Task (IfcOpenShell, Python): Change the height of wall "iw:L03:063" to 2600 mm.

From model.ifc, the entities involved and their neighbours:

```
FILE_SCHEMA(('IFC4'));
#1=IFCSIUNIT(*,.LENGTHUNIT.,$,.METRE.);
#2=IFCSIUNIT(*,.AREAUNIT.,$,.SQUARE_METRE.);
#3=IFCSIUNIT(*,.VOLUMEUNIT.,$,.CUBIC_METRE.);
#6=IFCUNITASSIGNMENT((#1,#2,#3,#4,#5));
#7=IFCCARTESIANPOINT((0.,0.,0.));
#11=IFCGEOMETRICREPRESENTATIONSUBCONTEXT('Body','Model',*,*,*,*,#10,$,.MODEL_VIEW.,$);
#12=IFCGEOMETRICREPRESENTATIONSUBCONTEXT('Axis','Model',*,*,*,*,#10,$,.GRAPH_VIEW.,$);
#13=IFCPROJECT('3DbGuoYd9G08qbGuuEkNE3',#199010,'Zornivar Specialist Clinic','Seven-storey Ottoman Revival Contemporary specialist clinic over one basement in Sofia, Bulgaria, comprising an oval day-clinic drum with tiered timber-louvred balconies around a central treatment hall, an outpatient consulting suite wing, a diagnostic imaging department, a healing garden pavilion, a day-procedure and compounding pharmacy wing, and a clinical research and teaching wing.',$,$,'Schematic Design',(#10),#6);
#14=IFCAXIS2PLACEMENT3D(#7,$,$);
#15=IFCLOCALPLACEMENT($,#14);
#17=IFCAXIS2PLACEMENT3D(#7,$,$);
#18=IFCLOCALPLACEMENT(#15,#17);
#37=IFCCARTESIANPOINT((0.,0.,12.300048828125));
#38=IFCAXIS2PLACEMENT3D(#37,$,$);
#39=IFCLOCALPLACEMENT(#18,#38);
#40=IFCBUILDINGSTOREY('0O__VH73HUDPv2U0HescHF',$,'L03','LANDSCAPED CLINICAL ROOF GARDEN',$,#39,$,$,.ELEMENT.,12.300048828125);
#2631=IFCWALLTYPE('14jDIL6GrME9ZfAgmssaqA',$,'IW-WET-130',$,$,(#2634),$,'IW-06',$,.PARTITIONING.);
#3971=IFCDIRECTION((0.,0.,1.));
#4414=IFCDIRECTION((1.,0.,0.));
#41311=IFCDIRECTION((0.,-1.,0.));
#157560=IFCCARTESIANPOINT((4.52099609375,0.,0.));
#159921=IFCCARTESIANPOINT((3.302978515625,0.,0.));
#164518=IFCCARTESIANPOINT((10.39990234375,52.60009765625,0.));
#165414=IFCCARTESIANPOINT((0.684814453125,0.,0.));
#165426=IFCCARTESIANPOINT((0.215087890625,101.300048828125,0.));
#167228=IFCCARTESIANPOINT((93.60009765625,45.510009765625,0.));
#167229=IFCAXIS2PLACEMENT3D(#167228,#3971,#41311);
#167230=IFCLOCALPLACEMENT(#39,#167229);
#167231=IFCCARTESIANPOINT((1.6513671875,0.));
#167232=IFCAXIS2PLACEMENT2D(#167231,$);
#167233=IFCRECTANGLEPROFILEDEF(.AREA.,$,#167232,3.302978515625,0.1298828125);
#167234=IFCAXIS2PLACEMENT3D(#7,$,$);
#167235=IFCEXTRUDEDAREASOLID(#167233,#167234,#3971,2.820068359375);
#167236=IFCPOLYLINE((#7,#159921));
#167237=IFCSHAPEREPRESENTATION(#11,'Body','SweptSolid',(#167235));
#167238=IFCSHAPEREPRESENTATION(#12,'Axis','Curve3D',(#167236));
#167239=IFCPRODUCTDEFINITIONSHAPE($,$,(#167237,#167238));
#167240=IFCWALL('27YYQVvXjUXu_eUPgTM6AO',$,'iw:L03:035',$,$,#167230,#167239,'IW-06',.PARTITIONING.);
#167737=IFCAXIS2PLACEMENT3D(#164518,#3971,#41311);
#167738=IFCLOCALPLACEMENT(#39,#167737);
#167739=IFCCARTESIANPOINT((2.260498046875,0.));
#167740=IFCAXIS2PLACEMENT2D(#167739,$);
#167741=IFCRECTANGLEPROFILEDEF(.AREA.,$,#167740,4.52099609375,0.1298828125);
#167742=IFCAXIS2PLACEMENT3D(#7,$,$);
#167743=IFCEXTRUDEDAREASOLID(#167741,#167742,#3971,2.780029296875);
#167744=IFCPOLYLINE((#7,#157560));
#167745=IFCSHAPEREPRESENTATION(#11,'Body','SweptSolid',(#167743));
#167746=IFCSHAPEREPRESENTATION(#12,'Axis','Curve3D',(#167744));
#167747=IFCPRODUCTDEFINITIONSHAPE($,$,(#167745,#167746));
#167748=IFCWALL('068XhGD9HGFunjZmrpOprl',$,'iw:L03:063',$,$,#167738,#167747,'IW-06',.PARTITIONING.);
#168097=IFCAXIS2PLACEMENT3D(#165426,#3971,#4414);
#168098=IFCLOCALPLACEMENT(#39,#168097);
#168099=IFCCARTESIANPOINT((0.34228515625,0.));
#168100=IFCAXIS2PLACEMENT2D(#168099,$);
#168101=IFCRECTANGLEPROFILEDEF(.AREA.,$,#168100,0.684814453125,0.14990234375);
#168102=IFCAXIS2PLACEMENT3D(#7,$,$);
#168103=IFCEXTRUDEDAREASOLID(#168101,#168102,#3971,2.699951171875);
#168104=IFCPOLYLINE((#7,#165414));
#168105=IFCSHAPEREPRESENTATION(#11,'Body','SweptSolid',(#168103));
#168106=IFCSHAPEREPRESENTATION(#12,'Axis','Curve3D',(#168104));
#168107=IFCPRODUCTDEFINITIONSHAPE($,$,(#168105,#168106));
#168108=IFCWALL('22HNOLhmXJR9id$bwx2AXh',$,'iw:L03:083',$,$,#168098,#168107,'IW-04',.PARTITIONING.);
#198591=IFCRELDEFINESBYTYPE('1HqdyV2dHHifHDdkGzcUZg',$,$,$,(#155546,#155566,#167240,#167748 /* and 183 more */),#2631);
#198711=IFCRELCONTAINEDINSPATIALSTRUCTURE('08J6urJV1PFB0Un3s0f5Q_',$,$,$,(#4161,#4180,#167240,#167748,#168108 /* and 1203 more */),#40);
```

```python
import ifcopenshell
import ifcopenshell.geom
import ifcopenshell.util.representation
import ifcopenshell.util.shape
import ifcopenshell.util.unit

model = ifcopenshell.open("model.ifc")
unit_scale = ifcopenshell.util.unit.calculate_unit_scale(model)
settings = ifcopenshell.geom.settings()


def volume(element):
    """Net volume in cubic metres, openings subtracted."""
    shape = ifcopenshell.geom.create_shape(settings, element)
    return ifcopenshell.util.shape.get_volume(shape.geometry)


wall = model.by_guid("068XhGD9HGFunjZmrpOprl")
before = volume(wall)

body = ifcopenshell.util.representation.get_representation(wall, "Model", "Body")
solid = body.Items[0]
old_height = solid.Depth
solid.Depth = 2.6 / unit_scale
after = volume(wall)

print(f"height {old_height:g} -> {solid.Depth:g}, volume {before:.3f} -> {after:.3f} m3")

model.write("model-out.ifc")
```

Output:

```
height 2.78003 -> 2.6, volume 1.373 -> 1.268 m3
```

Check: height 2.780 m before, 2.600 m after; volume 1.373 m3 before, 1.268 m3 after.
